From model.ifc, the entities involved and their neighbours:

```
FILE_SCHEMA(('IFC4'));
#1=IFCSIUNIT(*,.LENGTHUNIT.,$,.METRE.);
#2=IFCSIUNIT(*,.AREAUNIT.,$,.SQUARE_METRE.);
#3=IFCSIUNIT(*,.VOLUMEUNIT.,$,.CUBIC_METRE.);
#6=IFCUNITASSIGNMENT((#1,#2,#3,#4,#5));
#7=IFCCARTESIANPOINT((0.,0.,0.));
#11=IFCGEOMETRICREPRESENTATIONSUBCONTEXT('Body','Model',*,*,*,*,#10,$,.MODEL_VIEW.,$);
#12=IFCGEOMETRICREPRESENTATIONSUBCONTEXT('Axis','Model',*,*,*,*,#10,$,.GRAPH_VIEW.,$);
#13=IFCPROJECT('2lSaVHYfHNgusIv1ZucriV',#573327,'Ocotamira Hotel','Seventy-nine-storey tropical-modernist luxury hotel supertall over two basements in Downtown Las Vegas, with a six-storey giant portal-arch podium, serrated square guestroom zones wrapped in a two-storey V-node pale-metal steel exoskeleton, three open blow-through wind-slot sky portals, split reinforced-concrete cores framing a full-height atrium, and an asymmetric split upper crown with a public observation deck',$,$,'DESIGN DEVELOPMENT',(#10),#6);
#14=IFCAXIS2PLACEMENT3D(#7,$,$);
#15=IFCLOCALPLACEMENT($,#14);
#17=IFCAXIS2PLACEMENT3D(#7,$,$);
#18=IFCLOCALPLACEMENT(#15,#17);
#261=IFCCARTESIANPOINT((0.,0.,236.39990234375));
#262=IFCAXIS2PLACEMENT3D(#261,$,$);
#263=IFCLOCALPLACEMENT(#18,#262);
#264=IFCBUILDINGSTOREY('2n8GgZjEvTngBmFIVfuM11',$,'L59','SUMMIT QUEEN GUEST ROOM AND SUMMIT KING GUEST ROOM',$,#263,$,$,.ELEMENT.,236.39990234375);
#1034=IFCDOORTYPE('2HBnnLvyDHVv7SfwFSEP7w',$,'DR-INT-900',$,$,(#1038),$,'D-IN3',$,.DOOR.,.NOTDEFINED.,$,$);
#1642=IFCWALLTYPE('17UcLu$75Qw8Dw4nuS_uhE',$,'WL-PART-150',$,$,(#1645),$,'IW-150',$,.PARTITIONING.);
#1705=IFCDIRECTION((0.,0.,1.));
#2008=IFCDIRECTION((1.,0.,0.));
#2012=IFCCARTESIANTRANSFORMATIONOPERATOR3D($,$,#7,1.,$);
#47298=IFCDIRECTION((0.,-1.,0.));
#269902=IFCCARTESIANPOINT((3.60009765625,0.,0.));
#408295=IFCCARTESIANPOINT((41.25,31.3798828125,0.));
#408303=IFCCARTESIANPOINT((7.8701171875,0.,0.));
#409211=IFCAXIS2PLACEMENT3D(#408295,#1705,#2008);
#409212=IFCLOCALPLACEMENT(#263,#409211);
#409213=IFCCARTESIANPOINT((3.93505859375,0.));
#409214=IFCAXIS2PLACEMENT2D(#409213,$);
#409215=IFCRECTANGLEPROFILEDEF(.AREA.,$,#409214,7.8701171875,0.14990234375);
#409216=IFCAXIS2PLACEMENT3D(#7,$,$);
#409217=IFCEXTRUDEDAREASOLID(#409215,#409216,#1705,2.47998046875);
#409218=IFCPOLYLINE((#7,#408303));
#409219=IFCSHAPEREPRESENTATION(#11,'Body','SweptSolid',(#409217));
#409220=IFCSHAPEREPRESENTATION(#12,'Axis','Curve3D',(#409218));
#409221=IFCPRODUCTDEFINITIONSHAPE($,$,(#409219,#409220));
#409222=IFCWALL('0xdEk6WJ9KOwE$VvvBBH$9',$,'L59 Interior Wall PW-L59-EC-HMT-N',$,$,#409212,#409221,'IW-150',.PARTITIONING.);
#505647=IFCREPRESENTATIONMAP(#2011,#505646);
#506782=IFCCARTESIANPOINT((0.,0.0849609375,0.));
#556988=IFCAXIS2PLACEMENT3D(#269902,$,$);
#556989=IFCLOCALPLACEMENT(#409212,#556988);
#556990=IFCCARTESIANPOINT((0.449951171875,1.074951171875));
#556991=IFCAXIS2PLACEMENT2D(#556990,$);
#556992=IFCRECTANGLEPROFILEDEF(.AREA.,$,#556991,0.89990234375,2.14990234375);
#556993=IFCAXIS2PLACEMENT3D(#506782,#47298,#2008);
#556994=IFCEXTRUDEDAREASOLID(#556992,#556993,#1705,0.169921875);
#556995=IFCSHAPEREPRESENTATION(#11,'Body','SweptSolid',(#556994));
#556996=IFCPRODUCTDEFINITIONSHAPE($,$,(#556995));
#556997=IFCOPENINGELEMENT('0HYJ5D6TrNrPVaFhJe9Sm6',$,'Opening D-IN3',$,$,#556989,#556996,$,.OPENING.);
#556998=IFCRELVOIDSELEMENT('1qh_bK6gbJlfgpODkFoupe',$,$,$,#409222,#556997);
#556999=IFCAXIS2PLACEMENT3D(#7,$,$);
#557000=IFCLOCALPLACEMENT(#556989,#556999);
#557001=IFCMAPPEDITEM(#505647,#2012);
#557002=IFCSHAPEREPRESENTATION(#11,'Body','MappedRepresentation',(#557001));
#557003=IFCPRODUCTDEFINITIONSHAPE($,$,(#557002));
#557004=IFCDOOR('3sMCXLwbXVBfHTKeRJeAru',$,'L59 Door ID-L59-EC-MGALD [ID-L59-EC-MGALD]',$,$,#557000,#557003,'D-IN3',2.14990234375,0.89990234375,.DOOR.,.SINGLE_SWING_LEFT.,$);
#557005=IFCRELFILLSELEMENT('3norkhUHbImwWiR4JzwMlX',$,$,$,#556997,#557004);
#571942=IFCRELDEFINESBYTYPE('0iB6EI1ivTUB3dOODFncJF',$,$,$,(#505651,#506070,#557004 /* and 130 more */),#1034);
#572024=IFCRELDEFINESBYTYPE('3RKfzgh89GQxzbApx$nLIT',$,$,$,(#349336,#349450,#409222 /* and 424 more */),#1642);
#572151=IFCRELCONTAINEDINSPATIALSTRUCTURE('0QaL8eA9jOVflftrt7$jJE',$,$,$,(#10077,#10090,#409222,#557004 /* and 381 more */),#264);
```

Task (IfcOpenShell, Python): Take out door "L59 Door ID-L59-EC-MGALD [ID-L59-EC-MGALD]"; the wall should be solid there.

```python
import ifcopenshell
import ifcopenshell.api.feature
import ifcopenshell.api.root
import ifcopenshell.geom
import ifcopenshell.util.shape

model = ifcopenshell.open("model.ifc")
settings = ifcopenshell.geom.settings()


def volume(element):
    """Net volume in cubic metres, openings subtracted."""
    shape = ifcopenshell.geom.create_shape(settings, element)
    return ifcopenshell.util.shape.get_volume(shape.geometry)


door = model.by_id(557004)
opening = door.FillsVoids[0].RelatingOpeningElement
wall = opening.VoidsElements[0].RelatingBuildingElement
before = volume(wall)

ifcopenshell.api.root.remove_product(model, product=door)
ifcopenshell.api.feature.remove_feature(model, feature=opening)

after = volume(wall)

print(f"wall volume {before:.3f} -> {after:.3f} m3")

model.write("model-out.ifc")
```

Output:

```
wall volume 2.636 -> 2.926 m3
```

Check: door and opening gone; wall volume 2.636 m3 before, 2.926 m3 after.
